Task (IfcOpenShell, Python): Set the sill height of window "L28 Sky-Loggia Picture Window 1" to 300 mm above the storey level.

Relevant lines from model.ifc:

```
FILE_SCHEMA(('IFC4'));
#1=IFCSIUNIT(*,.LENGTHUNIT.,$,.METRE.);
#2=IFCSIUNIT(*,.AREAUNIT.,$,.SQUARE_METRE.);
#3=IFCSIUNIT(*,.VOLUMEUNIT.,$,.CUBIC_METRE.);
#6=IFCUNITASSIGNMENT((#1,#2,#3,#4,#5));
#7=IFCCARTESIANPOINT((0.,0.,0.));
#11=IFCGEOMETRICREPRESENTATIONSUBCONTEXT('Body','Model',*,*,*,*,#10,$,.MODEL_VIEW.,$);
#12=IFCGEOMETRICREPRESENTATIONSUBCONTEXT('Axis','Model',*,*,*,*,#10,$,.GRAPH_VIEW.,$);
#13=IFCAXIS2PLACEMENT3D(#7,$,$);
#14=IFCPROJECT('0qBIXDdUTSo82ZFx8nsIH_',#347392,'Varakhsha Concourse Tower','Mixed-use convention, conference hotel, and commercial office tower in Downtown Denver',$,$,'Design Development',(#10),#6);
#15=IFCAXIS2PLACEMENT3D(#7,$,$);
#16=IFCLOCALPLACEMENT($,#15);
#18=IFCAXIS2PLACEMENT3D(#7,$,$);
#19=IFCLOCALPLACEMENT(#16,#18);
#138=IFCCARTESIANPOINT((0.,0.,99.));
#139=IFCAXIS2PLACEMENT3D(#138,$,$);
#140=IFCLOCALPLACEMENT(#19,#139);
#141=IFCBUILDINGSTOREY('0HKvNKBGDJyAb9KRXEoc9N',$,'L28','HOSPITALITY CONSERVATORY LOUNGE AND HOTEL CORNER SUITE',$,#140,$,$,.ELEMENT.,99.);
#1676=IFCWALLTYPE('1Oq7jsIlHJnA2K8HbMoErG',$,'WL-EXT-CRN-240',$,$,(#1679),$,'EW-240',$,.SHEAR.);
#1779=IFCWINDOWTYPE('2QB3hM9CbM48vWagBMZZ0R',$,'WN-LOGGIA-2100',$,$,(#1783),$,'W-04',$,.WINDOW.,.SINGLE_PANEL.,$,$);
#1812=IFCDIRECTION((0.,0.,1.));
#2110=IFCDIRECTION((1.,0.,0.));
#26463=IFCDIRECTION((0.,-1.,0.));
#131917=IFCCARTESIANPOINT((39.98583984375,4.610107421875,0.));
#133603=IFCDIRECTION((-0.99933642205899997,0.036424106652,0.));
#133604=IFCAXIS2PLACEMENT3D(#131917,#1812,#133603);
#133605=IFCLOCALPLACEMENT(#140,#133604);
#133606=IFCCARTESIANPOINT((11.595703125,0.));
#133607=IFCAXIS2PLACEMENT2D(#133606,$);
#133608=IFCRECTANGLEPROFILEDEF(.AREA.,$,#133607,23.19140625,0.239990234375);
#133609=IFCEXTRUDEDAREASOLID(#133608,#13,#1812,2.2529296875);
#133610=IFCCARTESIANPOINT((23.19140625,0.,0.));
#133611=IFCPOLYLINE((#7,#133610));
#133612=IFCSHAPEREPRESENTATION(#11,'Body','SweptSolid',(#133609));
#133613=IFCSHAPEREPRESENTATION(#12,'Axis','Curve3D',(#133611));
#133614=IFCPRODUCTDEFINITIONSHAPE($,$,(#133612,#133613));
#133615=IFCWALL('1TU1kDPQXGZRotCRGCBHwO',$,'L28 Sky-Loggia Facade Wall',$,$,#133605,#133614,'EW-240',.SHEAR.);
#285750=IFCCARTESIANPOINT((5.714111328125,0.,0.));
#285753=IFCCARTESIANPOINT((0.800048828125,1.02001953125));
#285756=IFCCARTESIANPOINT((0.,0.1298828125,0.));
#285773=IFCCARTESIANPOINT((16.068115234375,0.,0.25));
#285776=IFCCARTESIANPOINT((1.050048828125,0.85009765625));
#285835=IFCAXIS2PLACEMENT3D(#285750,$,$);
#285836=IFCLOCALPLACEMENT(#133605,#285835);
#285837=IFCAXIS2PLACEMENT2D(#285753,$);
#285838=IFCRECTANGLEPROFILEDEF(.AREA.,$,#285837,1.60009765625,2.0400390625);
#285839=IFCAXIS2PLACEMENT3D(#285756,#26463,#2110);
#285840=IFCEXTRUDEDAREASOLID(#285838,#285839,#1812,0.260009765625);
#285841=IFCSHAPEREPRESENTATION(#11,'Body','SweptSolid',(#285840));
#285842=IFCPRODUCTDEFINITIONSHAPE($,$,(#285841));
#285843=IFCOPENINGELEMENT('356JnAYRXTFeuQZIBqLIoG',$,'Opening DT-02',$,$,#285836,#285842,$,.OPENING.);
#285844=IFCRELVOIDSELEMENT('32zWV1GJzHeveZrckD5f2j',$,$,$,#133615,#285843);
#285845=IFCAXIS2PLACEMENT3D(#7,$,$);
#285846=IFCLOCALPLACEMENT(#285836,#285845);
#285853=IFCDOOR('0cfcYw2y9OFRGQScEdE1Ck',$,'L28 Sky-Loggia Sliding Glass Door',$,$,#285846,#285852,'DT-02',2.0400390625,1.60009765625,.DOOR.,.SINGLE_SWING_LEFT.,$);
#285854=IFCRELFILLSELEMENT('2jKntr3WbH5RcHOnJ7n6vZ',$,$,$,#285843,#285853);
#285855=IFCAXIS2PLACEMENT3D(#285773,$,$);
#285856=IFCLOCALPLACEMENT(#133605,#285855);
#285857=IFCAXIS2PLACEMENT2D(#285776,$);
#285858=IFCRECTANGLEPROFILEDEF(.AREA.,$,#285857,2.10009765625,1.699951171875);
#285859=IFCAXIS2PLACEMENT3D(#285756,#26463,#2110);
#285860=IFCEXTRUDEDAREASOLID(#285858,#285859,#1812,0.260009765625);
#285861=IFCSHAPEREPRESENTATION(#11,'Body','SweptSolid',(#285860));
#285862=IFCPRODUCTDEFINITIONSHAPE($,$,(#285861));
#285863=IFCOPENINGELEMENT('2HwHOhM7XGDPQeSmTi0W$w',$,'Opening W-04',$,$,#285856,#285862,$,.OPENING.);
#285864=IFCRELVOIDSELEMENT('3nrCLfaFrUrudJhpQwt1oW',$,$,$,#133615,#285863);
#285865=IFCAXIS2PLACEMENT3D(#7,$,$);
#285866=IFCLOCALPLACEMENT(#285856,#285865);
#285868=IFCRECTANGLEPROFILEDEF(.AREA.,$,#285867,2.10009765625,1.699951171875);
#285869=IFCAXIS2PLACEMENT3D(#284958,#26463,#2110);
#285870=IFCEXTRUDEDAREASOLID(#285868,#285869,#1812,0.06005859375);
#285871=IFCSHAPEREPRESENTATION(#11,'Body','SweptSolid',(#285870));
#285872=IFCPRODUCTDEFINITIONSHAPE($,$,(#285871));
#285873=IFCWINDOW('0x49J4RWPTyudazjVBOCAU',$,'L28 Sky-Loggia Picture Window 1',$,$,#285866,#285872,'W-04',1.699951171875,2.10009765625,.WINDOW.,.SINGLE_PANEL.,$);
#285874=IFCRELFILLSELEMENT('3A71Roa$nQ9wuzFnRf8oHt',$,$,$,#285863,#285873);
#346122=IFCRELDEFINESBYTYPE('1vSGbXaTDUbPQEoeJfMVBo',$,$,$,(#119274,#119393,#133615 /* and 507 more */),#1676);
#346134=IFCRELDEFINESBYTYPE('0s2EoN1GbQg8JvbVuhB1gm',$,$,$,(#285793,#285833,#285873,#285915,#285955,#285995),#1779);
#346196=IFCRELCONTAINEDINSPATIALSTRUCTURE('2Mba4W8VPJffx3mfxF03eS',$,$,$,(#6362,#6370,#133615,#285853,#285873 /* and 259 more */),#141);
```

```python
import numpy as np
import ifcopenshell
import ifcopenshell.api.geometry
import ifcopenshell.geom
import ifcopenshell.util.element
import ifcopenshell.util.placement
import ifcopenshell.util.shape
import ifcopenshell.util.unit

model = ifcopenshell.open("model.ifc")
unit_scale = ifcopenshell.util.unit.calculate_unit_scale(model)

window = model.by_guid("0x49J4RWPTyudazjVBOCAU")
opening = window.FillsVoids[0].RelatingOpeningElement
storey = ifcopenshell.util.element.get_container(window, ifc_class="IfcBuildingStorey")
level = ifcopenshell.util.placement.get_local_placement(storey.ObjectPlacement)[2, 3]

# The opening's origin need not be at the sill, so measure its lowest point.
shape = ifcopenshell.geom.create_shape(ifcopenshell.geom.settings(), opening)
bottom = ifcopenshell.util.shape.get_shape_bottom_elevation(shape, shape.geometry) / unit_scale
dz = level + 0.3 / unit_scale - bottom

shift = np.array([0.0, 0.0, dz])
# The window is placed relative to its opening, so it follows when the opening moves.
matrix = ifcopenshell.util.placement.get_local_placement(opening.ObjectPlacement)
matrix[:3, 3] += shift
ifcopenshell.api.geometry.edit_object_placement(
    model, product=opening, matrix=matrix, is_si=False, should_transform_children=True
)

print(f"moved by {dz * unit_scale:+.3f} m")

model.write("model_v2.ifc")
```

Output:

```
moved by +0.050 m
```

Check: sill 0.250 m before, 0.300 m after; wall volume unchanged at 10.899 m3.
